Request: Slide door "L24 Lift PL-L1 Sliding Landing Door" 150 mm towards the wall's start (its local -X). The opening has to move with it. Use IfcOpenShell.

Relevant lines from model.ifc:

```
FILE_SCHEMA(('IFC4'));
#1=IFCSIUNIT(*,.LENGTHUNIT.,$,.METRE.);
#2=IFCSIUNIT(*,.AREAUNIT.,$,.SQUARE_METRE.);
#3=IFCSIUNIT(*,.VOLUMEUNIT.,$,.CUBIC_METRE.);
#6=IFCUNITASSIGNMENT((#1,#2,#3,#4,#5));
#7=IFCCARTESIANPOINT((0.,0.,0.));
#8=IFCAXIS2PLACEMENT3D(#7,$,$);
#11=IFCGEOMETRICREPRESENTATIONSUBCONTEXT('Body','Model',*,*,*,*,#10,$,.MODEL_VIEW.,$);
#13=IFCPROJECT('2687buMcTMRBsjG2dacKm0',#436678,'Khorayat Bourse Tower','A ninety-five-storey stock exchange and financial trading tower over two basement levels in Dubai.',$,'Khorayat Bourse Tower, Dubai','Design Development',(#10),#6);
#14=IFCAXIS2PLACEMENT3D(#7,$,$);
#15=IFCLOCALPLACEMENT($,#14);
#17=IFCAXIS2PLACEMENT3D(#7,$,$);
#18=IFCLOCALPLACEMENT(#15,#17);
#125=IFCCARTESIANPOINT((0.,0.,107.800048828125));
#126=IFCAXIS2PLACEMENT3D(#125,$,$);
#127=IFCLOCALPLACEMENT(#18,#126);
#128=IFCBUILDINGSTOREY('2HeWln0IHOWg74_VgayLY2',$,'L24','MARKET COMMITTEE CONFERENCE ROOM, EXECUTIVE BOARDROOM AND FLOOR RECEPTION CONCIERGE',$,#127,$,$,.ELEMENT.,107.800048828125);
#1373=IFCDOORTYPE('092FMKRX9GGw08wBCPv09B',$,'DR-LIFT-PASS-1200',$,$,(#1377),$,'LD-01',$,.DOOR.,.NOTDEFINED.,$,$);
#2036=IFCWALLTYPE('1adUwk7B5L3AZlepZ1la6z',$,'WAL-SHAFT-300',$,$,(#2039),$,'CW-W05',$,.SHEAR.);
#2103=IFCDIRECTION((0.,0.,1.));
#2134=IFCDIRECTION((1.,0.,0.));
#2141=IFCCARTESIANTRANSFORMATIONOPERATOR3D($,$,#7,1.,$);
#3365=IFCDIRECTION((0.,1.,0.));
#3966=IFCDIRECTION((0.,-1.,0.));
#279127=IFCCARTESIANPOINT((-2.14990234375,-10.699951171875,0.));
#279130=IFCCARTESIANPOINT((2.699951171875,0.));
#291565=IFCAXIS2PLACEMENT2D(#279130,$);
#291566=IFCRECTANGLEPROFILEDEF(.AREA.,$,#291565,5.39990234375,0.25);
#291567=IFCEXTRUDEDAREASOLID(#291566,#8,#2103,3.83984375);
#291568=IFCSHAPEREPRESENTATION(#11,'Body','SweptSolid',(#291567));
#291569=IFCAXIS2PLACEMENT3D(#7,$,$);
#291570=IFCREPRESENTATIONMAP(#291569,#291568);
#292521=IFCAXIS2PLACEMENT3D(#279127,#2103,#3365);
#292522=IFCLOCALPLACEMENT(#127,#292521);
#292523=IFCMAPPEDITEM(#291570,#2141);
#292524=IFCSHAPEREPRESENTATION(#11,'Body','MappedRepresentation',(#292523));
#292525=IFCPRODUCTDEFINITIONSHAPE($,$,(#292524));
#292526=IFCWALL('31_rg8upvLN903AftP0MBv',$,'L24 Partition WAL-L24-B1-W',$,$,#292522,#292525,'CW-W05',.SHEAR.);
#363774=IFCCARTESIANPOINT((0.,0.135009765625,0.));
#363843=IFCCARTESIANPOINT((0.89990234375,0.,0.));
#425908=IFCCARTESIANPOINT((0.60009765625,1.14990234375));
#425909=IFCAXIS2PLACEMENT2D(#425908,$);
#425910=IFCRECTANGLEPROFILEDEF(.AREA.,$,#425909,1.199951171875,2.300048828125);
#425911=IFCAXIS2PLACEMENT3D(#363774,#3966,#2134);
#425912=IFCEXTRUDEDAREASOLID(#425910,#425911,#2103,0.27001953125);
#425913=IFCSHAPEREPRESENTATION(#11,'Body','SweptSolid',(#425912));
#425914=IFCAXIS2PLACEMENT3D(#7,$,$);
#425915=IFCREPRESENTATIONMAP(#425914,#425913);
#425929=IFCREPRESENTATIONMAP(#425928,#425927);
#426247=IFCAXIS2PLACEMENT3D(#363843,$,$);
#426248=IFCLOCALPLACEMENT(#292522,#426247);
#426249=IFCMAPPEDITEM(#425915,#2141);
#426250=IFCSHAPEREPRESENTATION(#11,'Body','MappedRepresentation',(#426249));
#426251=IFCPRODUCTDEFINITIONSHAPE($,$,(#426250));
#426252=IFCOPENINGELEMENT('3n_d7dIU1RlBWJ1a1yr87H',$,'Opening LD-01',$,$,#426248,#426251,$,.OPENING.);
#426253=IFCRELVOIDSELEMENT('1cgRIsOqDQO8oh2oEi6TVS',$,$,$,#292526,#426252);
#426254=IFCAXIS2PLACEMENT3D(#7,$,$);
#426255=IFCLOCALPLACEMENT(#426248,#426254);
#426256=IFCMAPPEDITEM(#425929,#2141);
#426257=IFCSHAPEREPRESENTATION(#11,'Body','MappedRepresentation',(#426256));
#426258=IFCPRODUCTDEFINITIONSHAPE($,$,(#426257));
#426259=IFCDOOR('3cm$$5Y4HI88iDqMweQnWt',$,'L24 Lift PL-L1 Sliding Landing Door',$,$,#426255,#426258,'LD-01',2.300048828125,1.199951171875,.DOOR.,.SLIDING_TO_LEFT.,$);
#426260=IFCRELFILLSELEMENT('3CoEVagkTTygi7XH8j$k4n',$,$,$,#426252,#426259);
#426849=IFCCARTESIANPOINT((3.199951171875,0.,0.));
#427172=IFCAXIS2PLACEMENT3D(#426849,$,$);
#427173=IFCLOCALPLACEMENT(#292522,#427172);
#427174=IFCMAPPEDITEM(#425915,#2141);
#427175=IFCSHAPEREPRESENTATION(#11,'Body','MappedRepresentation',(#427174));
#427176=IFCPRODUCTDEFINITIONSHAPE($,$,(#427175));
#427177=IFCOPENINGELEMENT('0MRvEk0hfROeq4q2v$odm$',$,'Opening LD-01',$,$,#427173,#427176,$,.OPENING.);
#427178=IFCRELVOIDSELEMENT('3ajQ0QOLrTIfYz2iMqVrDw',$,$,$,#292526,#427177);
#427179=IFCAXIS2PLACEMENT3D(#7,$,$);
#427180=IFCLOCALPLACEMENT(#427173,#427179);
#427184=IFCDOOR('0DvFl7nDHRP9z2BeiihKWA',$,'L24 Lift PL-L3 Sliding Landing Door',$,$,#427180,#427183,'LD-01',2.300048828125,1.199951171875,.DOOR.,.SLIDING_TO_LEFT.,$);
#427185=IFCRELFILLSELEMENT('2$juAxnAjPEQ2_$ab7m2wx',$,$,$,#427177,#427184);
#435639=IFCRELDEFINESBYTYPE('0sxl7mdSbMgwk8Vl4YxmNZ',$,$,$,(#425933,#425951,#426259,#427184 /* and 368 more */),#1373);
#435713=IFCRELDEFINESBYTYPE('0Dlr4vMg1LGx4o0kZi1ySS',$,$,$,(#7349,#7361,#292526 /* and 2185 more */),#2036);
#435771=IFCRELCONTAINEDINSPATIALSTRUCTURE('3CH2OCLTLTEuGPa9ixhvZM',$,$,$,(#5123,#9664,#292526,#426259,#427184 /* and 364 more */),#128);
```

```python
import ifcopenshell
import ifcopenshell.api.geometry
import ifcopenshell.util.placement
import ifcopenshell.util.unit

model = ifcopenshell.open("model.ifc")
unit_scale = ifcopenshell.util.unit.calculate_unit_scale(model)

door = model.by_guid("3cm$$5Y4HI88iDqMweQnWt")
opening = door.FillsVoids[0].RelatingOpeningElement
wall = opening.VoidsElements[0].RelatingBuildingElement

wall_matrix = ifcopenshell.util.placement.get_local_placement(wall.ObjectPlacement)
shift = wall_matrix[:3, 0] * -0.15 / unit_scale
before = ifcopenshell.util.placement.get_local_placement(door.ObjectPlacement)[:3, 3].copy()

# The door is placed relative to its opening, so it follows when the opening moves.
matrix = ifcopenshell.util.placement.get_local_placement(opening.ObjectPlacement)
matrix[:3, 3] += shift
ifcopenshell.api.geometry.edit_object_placement(
    model, product=opening, matrix=matrix, is_si=False, should_transform_children=True
)

after = ifcopenshell.util.placement.get_local_placement(door.ObjectPlacement)[:3, 3]
print("door moved by", (after - before).round(3) + 0.0)

model.write("model_rev.ifc")
```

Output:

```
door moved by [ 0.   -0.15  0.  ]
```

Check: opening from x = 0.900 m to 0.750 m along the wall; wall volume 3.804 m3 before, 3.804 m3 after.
